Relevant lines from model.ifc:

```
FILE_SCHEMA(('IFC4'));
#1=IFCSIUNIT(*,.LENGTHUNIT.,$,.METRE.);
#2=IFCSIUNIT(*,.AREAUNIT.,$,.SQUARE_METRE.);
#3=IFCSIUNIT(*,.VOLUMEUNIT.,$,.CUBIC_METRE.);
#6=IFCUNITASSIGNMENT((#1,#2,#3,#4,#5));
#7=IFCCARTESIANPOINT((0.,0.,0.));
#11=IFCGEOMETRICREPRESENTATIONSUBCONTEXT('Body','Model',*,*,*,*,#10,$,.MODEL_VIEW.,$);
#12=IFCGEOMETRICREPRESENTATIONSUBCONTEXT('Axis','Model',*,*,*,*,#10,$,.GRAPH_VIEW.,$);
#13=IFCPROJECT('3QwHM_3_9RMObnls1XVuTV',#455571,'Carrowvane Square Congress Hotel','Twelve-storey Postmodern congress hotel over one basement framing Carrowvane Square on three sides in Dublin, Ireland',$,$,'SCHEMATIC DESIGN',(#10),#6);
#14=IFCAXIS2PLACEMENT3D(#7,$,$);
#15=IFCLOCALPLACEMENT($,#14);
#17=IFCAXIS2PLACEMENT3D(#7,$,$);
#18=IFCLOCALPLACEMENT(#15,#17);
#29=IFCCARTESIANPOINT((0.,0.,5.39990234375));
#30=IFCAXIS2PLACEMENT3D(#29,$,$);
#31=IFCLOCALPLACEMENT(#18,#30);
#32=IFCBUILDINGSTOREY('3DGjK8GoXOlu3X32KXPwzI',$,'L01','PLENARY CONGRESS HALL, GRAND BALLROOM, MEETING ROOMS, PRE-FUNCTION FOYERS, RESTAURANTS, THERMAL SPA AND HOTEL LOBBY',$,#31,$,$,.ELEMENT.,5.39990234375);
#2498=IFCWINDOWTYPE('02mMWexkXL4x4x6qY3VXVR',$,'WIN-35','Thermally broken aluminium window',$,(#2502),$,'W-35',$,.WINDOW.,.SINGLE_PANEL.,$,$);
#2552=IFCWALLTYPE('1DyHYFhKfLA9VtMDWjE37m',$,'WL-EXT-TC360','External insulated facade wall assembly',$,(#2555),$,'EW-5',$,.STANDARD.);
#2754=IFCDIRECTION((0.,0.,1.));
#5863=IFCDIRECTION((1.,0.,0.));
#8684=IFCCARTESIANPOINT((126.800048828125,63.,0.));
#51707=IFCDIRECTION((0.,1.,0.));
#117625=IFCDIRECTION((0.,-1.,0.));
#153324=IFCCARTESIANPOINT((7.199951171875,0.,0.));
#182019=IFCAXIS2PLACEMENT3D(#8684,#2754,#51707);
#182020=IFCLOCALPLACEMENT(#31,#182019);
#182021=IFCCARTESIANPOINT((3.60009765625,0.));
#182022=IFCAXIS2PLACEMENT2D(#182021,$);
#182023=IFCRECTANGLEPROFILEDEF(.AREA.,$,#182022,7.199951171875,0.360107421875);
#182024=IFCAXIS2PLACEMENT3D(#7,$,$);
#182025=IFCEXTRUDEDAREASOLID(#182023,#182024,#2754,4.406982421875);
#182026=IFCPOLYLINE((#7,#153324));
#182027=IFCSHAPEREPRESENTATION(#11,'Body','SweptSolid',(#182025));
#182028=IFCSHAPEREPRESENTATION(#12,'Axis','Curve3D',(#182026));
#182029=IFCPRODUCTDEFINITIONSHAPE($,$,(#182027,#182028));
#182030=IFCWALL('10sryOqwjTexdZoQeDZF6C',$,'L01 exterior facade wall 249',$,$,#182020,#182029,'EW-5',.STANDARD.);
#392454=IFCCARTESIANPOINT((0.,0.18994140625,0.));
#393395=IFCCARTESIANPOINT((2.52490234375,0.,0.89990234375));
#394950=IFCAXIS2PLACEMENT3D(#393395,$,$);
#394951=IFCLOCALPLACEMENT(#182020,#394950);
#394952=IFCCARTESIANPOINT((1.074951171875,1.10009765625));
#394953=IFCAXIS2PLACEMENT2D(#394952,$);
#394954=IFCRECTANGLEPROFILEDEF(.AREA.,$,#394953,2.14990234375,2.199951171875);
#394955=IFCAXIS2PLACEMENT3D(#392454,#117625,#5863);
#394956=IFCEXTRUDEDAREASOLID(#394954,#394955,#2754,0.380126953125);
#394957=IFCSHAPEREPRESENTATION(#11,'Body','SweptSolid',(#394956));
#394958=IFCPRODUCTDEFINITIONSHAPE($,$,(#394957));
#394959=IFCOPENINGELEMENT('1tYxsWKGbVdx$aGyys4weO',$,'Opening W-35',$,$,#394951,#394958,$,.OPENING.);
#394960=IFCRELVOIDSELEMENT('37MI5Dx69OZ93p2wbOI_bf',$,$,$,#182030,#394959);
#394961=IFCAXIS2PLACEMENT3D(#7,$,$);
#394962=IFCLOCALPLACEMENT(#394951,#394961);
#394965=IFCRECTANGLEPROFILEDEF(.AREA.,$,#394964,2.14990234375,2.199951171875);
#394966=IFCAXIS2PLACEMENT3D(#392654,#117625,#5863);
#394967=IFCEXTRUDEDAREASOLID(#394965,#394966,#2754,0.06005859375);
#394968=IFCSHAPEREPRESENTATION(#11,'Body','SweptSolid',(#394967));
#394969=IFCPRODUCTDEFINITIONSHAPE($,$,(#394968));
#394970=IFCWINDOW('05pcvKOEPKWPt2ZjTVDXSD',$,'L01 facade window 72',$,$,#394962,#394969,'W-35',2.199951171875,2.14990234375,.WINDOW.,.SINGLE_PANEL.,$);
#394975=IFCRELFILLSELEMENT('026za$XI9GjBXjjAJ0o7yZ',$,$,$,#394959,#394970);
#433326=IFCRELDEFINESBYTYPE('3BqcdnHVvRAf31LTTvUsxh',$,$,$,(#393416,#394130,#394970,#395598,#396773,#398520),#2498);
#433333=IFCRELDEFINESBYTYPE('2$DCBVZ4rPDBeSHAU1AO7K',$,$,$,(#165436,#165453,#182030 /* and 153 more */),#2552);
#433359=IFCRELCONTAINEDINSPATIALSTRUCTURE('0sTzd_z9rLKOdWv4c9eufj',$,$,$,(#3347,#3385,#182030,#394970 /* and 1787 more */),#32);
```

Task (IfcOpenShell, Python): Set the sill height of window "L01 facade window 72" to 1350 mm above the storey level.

```python
import numpy as np
import ifcopenshell
import ifcopenshell.api.geometry
import ifcopenshell.geom
import ifcopenshell.util.element
import ifcopenshell.util.placement
import ifcopenshell.util.shape
import ifcopenshell.util.unit

model = ifcopenshell.open("model.ifc")
unit_scale = ifcopenshell.util.unit.calculate_unit_scale(model)

window = model.by_id(394970)
opening = window.FillsVoids[0].RelatingOpeningElement
storey = ifcopenshell.util.element.get_container(window, ifc_class="IfcBuildingStorey")
level = ifcopenshell.util.placement.get_local_placement(storey.ObjectPlacement)[2, 3]

# The opening's origin need not be at the sill, so measure its lowest point.
shape = ifcopenshell.geom.create_shape(ifcopenshell.geom.settings(), opening)
bottom = ifcopenshell.util.shape.get_shape_bottom_elevation(shape, shape.geometry) / unit_scale
dz = level + 1.35 - bottom

shift = np.array([0.0, 0.0, dz])
# The window is placed relative to its opening, so it follows when the opening moves.
matrix = ifcopenshell.util.placement.get_local_placement(opening.ObjectPlacement)
matrix[:3, 3] += shift
ifcopenshell.api.geometry.edit_object_placement(
    model, product=opening, matrix=matrix, is_si=False, should_transform_children=True
)

print(f"moved by {dz * unit_scale:+.3f} m")

model.write("model_updated.ifc")
```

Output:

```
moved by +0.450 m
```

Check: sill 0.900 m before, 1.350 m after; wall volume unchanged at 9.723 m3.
